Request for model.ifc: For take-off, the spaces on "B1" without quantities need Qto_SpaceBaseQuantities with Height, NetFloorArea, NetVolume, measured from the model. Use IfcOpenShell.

First a look at what the model holds.

```python
import ifcopenshell
import ifcopenshell.util.element
import ifcopenshell.util.unit

model = ifcopenshell.open("model.ifc")
print(model.schema)
for unit_type in ("LENGTHUNIT", "AREAUNIT", "VOLUMEUNIT"):
    print(unit_type, ifcopenshell.util.unit.calculate_unit_scale(model, unit_type))
storey = next(s for s in model.by_type("IfcBuildingStorey") if s.Name == "B1")
spaces = [e for e in ifcopenshell.util.element.get_decomposition(storey) if e.is_a("IfcSpace")]
for e in sorted(spaces, key=lambda e: e.id()):
    print(e.id(), e.is_a(), e.Name, list(ifcopenshell.util.element.get_psets(e, qtos_only=True)), sep=" | ")
```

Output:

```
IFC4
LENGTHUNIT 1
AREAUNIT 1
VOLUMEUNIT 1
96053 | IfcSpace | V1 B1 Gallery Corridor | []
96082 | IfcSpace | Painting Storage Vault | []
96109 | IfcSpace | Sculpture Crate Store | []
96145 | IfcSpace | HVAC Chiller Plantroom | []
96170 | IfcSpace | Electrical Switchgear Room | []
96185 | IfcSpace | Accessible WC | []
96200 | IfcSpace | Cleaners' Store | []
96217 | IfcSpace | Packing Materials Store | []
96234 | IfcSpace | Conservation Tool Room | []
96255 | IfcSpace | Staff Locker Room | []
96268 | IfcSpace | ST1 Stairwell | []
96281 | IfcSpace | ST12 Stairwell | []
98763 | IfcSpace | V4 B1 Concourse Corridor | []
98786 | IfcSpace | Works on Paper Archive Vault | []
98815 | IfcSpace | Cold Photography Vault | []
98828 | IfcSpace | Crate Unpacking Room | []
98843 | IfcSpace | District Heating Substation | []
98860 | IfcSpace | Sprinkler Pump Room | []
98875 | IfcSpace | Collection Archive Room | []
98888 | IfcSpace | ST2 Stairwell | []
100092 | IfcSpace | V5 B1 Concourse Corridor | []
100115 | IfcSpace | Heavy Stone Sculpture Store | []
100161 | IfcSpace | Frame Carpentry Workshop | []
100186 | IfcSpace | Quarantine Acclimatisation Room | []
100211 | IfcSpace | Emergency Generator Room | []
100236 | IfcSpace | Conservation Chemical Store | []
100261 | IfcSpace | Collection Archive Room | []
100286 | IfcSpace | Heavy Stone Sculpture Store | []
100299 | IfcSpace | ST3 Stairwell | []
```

```python
import ifcopenshell
import ifcopenshell.api.pset
import ifcopenshell.geom
import ifcopenshell.util.element
import ifcopenshell.util.shape
import ifcopenshell.util.unit

model = ifcopenshell.open("model.ifc")
unit_scale = ifcopenshell.util.unit.calculate_unit_scale(model)
area_scale = ifcopenshell.util.unit.calculate_unit_scale(model, "AREAUNIT")
volume_scale = ifcopenshell.util.unit.calculate_unit_scale(model, "VOLUMEUNIT")
settings = ifcopenshell.geom.settings()

storey = next(s for s in model.by_type("IfcBuildingStorey") if s.Name == "B1")
spaces = [e for e in ifcopenshell.util.element.get_decomposition(storey) if e.is_a("IfcSpace")]

for e in sorted(spaces, key=lambda e: e.id()):
    if ifcopenshell.util.element.get_psets(e, qtos_only=True, should_inherit=False):
        continue
    # Geometry comes back in metres, in the element's own axes.
    shape = ifcopenshell.geom.create_shape(settings, e)
    values = {
        "Height": ifcopenshell.util.shape.get_z(shape.geometry) / unit_scale,
        "NetFloorArea": ifcopenshell.util.shape.get_footprint_area(shape.geometry) / area_scale,
        "NetVolume": ifcopenshell.util.shape.get_volume(shape.geometry) / volume_scale,
    }
    qto = ifcopenshell.api.pset.add_qto(model, product=e, name="Qto_SpaceBaseQuantities")
    ifcopenshell.api.pset.edit_qto(model, qto=qto, properties=values)
    print(e.id(), {k: round(v, 3) for k, v in values.items()})

model.write("model-out.ifc")
```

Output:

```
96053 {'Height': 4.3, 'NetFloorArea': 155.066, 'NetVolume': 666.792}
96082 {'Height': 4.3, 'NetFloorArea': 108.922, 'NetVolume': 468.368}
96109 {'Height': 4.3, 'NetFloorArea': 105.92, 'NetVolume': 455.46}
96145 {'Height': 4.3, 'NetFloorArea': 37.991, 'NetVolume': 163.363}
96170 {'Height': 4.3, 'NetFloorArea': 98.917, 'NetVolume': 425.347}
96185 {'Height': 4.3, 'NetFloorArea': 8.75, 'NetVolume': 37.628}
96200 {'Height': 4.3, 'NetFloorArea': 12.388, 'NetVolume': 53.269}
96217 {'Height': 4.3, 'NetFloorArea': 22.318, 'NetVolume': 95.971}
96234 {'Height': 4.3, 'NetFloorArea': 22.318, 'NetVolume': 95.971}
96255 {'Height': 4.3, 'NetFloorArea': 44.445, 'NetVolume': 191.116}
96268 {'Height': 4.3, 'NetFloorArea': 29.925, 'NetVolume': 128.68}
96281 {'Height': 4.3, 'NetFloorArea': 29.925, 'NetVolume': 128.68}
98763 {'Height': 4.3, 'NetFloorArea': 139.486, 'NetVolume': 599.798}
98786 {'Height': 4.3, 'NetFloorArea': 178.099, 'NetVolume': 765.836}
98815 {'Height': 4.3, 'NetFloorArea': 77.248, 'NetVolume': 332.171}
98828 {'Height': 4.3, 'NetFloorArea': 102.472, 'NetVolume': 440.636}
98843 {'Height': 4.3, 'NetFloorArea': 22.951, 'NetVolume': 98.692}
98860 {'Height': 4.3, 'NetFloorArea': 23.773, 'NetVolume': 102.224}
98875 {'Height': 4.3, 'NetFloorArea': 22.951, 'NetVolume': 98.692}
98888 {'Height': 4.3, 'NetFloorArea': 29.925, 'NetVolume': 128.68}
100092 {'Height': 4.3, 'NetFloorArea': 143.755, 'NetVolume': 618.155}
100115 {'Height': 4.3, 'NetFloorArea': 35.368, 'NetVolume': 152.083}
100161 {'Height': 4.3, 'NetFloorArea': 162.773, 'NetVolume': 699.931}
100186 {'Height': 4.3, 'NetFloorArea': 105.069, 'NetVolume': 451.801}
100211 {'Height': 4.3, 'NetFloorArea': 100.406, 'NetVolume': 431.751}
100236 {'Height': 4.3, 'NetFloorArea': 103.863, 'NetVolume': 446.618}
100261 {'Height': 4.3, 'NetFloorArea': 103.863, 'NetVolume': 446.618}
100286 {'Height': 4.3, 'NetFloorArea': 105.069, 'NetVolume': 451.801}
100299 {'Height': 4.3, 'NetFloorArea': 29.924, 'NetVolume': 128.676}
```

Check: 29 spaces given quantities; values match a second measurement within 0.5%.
